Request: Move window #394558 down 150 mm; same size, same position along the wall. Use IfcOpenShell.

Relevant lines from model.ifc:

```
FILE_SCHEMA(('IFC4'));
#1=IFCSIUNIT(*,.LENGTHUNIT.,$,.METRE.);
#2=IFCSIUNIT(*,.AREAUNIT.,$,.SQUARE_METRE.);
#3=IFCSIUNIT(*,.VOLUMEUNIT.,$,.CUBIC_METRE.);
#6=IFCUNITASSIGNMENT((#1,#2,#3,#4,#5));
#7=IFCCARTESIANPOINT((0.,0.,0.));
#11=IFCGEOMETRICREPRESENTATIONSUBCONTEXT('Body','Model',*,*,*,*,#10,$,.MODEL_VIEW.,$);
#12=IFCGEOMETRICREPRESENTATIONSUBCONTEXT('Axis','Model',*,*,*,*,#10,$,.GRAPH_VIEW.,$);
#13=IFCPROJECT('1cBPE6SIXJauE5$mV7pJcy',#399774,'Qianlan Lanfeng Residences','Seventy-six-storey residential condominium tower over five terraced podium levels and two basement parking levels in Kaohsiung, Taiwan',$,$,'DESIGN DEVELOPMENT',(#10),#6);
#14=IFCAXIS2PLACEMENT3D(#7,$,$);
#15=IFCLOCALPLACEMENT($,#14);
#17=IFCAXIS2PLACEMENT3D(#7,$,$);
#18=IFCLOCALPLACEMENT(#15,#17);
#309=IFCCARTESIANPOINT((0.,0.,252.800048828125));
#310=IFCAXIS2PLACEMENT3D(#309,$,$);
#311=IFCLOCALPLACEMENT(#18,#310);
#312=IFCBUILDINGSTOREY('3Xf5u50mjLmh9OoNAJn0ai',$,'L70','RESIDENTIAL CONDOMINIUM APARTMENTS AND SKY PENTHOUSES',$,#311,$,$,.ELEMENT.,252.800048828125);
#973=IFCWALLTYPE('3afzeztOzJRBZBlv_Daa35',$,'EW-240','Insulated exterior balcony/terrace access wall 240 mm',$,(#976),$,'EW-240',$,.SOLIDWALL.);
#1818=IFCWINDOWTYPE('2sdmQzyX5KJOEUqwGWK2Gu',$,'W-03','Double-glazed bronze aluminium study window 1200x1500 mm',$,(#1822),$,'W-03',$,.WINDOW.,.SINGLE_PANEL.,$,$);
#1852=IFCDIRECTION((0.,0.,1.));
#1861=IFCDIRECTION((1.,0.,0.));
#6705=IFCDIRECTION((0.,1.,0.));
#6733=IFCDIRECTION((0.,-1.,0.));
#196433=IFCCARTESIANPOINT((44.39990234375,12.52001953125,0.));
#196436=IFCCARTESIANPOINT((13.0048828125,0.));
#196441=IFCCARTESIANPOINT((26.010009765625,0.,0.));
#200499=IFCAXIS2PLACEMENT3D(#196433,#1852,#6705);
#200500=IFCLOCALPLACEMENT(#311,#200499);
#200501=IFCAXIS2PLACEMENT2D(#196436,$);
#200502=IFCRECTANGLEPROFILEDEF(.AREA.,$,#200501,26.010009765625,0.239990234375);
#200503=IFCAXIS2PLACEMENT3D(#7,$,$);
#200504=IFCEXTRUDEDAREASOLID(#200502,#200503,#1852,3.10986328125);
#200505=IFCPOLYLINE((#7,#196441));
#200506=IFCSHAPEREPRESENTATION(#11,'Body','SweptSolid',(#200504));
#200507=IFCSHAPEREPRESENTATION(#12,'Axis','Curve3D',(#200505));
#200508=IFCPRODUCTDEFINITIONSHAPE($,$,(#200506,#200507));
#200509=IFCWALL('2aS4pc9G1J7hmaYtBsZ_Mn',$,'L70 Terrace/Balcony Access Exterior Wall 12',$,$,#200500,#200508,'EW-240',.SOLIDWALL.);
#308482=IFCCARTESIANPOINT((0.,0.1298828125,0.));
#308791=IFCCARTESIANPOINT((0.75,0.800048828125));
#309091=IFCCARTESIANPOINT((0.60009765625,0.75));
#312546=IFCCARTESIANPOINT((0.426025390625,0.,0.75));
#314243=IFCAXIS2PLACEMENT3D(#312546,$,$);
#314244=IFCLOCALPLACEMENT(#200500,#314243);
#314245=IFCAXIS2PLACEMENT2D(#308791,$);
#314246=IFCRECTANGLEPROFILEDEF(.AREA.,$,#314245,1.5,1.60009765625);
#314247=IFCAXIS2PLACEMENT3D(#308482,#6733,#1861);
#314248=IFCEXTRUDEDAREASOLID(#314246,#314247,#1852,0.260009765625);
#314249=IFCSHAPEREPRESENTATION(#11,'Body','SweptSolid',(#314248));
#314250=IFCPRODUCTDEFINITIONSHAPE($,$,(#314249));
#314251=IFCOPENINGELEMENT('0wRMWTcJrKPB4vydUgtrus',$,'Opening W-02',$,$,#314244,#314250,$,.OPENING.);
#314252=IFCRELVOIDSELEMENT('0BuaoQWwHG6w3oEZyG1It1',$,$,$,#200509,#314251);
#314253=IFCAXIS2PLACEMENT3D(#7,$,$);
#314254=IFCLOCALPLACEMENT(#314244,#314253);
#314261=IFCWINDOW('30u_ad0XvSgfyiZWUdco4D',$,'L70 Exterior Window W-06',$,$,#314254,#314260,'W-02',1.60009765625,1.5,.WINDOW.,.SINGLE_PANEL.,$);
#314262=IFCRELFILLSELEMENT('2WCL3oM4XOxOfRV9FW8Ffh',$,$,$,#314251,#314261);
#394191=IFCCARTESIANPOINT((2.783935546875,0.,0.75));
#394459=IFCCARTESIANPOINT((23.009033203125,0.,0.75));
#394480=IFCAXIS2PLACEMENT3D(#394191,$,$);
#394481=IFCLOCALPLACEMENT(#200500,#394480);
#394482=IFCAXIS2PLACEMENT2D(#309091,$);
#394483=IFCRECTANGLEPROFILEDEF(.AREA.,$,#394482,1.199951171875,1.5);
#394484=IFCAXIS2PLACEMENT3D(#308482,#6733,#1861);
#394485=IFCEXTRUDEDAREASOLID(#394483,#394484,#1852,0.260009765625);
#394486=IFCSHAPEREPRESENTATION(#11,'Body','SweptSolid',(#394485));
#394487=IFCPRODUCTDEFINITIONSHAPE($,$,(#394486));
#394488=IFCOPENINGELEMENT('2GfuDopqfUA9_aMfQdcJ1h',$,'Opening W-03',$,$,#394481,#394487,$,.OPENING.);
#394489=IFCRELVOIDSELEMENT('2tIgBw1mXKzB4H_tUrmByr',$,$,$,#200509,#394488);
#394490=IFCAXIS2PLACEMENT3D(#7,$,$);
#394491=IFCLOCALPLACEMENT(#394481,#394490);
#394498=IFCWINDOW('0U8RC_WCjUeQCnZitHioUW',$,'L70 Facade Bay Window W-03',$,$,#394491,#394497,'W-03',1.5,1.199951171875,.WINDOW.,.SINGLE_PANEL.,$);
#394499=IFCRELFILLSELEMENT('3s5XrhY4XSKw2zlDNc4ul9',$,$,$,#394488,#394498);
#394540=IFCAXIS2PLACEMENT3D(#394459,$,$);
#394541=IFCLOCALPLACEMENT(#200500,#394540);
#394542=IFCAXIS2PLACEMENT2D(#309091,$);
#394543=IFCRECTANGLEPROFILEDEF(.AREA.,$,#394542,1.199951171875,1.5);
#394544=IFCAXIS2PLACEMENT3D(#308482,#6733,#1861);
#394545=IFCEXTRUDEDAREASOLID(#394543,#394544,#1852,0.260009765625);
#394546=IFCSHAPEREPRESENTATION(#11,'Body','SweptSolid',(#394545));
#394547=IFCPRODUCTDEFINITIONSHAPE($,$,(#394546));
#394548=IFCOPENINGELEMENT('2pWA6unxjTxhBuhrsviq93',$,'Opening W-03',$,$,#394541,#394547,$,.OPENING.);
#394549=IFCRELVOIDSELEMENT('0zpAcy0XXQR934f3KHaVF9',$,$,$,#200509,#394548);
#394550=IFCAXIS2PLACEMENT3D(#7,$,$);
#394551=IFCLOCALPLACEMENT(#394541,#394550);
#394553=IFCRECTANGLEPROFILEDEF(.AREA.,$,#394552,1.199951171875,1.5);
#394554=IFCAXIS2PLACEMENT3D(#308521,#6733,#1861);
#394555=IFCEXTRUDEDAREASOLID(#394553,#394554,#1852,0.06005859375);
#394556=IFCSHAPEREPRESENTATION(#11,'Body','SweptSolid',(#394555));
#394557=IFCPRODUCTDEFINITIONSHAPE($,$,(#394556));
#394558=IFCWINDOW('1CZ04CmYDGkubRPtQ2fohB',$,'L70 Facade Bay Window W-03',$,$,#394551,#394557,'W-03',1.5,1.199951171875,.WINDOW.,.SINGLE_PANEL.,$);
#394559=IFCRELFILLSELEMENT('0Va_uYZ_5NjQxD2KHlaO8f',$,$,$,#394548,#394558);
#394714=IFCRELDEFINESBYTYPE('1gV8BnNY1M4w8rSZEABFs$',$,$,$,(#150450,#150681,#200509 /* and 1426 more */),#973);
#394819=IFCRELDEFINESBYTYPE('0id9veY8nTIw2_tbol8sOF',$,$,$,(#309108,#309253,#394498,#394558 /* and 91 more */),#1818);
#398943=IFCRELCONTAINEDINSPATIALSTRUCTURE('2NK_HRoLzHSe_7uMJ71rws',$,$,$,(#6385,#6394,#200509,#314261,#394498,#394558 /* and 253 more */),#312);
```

```python
import numpy as np
import ifcopenshell
import ifcopenshell.api.geometry
import ifcopenshell.util.placement
import ifcopenshell.util.unit

model = ifcopenshell.open("model.ifc")
unit_scale = ifcopenshell.util.unit.calculate_unit_scale(model)

window = model.by_id(394558)
opening = window.FillsVoids[0].RelatingOpeningElement
dz = -0.15

shift = np.array([0.0, 0.0, dz])
# The window is placed relative to its opening, so it follows when the opening moves.
matrix = ifcopenshell.util.placement.get_local_placement(opening.ObjectPlacement)
matrix[:3, 3] += shift
ifcopenshell.api.geometry.edit_object_placement(
    model, product=opening, matrix=matrix, is_si=False, should_transform_children=True
)

print(f"moved by {dz * unit_scale:+.3f} m")

model.write("model-out.ifc")
```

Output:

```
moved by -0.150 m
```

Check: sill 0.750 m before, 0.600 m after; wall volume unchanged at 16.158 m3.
